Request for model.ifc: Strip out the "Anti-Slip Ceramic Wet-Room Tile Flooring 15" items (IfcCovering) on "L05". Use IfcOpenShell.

First a look at what the model holds.

```python
import ifcopenshell
import ifcopenshell.util.element

model = ifcopenshell.open("model.ifc")
print(model.schema)
storey = next(s for s in model.by_type("IfcBuildingStorey") if s.Name == "L05")
coverings = [e for e in ifcopenshell.util.element.get_decomposition(storey) if e.is_a("IfcCovering")]
seen = {}
for e in coverings:
    element_type = ifcopenshell.util.element.get_type(e)
    name = element_type.Name if element_type not in (None, e) else None
    seen[name] = seen.get(name, 0) + 1
for name, count in sorted(seen.items(), key=str):
    print(count, "x", name)
```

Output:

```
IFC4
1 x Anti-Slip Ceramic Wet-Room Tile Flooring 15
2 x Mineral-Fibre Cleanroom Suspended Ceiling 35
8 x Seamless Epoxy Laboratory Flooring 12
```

```python
import ifcopenshell
import ifcopenshell.api.root
import ifcopenshell.util.element

model = ifcopenshell.open("model.ifc")

storey = next(s for s in model.by_type("IfcBuildingStorey") if s.Name == "L05")
coverings = [e for e in ifcopenshell.util.element.get_decomposition(storey) if e.is_a("IfcCovering")]
targets = [e for e in coverings if (t := ifcopenshell.util.element.get_type(e)) not in (None, e) and t.Name == "Anti-Slip Ceramic Wet-Room Tile Flooring 15"]

for e in targets:
    ifcopenshell.api.root.remove_product(model, product=e)
print(len(targets), "removed")

model.write("model-out.ifc")
```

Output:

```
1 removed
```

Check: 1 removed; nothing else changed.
